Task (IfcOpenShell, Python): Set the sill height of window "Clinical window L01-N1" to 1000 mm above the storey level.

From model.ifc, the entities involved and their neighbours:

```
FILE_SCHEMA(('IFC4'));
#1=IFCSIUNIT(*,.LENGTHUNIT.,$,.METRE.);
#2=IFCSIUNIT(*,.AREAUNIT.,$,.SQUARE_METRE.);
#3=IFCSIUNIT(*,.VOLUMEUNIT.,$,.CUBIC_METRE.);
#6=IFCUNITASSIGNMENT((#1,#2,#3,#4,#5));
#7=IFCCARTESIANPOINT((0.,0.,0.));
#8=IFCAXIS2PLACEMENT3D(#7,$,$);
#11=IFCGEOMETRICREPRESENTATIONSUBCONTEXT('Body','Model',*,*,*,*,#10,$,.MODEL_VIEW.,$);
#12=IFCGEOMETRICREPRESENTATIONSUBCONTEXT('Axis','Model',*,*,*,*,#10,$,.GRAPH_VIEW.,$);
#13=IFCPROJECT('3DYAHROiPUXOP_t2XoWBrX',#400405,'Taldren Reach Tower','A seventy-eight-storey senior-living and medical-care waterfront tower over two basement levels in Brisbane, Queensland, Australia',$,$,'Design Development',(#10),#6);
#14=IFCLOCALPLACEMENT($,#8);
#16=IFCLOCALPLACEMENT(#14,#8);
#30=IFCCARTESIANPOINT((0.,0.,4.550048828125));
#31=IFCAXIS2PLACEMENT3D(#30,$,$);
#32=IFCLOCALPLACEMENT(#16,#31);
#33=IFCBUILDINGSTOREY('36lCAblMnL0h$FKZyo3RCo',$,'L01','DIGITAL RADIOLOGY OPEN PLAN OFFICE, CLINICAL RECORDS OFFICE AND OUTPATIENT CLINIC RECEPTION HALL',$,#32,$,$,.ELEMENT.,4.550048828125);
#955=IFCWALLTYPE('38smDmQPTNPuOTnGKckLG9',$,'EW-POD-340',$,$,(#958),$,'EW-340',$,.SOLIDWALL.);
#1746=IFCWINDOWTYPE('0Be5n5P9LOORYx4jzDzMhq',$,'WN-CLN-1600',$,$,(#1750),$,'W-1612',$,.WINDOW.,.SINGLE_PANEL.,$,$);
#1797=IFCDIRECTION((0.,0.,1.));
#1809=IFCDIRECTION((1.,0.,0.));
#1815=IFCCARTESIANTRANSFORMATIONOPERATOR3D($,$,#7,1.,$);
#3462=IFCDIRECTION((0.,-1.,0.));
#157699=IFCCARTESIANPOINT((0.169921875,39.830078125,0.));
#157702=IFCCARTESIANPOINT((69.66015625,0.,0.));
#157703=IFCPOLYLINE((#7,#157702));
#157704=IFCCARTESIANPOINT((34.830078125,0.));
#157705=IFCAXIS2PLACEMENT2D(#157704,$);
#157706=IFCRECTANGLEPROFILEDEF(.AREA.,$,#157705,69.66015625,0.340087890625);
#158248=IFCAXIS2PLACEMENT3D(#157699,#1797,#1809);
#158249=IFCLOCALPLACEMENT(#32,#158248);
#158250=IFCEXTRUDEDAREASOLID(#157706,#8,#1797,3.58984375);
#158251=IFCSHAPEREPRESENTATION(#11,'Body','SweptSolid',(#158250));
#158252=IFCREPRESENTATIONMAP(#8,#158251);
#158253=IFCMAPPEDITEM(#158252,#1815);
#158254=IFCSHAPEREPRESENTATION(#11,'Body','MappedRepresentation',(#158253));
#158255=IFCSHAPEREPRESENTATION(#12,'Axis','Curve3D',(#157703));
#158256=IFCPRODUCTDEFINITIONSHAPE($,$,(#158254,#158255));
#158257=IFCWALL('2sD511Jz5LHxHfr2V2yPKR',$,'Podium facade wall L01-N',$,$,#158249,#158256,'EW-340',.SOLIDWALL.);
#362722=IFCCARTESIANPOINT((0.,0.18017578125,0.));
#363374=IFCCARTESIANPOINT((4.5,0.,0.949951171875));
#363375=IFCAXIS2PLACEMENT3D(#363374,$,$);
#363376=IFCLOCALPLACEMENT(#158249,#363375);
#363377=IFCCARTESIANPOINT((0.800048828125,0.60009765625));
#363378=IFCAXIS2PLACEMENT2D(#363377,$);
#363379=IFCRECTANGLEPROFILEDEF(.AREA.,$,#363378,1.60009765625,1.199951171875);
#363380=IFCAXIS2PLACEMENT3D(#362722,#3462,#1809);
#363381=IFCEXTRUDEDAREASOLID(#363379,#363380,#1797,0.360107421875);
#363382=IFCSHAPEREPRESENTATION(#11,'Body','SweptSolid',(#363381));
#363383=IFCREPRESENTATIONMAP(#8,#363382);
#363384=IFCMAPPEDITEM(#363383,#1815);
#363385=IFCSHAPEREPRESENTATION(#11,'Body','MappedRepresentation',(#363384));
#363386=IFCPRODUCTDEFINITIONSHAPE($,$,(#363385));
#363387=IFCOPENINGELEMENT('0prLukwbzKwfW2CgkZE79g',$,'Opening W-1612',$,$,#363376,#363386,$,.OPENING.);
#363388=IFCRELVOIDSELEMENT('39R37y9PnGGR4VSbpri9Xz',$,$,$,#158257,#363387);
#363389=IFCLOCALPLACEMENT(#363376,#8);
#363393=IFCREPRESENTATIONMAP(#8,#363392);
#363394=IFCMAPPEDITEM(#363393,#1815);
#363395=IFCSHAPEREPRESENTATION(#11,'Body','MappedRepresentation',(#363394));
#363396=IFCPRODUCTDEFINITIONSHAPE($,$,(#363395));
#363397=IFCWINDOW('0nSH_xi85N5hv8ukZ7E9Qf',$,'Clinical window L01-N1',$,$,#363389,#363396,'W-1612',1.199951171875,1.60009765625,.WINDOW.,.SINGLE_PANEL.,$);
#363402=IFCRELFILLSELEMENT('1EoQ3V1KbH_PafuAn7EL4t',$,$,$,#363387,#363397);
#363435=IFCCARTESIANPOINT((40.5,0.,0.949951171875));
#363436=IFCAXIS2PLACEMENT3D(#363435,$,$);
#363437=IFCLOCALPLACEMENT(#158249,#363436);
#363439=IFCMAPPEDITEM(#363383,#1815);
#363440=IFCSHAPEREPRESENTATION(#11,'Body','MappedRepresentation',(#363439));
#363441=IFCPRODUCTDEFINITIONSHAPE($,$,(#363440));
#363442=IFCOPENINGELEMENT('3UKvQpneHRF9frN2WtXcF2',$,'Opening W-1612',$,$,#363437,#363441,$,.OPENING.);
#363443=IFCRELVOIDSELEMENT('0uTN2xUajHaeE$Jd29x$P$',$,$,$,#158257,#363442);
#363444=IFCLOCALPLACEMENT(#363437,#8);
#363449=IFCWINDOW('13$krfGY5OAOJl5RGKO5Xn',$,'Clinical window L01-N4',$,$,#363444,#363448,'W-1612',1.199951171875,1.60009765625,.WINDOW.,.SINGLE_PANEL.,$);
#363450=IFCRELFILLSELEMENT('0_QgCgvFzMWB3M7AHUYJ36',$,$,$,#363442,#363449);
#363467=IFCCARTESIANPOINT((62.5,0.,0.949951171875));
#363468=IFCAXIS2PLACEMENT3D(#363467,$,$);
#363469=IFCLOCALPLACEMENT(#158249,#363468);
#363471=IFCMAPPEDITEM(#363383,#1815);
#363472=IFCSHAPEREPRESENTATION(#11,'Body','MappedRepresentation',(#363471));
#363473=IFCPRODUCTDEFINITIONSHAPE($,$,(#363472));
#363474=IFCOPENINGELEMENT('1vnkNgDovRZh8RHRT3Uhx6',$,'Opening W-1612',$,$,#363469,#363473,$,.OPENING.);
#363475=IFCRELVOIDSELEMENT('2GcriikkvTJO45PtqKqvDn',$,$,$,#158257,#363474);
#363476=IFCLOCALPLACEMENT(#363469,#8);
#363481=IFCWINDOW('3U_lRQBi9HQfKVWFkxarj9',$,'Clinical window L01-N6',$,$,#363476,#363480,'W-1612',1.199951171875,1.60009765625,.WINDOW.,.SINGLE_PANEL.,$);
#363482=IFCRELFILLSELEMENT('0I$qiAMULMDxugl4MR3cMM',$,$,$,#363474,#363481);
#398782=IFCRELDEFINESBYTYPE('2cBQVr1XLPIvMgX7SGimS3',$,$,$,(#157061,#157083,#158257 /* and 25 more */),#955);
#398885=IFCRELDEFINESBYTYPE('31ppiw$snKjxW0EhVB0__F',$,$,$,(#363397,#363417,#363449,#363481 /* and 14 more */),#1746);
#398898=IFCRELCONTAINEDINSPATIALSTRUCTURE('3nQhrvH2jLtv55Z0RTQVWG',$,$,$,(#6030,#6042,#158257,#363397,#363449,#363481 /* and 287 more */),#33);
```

```python
import numpy as np
import ifcopenshell
import ifcopenshell.api.geometry
import ifcopenshell.geom
import ifcopenshell.util.element
import ifcopenshell.util.placement
import ifcopenshell.util.shape
import ifcopenshell.util.unit

model = ifcopenshell.open("model.ifc")
unit_scale = ifcopenshell.util.unit.calculate_unit_scale(model)

window = model.by_guid("0nSH_xi85N5hv8ukZ7E9Qf")
opening = window.FillsVoids[0].RelatingOpeningElement
storey = ifcopenshell.util.element.get_container(window, ifc_class="IfcBuildingStorey")
level = ifcopenshell.util.placement.get_local_placement(storey.ObjectPlacement)[2, 3]

# The opening's origin need not be at the sill, so measure its lowest point.
shape = ifcopenshell.geom.create_shape(ifcopenshell.geom.settings(), opening)
bottom = ifcopenshell.util.shape.get_shape_bottom_elevation(shape, shape.geometry) / unit_scale
dz = level + 1.0 - bottom

shift = np.array([0.0, 0.0, dz])
# The window is placed relative to its opening, so it follows when the opening moves.
matrix = ifcopenshell.util.placement.get_local_placement(opening.ObjectPlacement)
matrix[:3, 3] += shift
ifcopenshell.api.geometry.edit_object_placement(
    model, product=opening, matrix=matrix, is_si=False, should_transform_children=True
)

print(f"moved by {dz * unit_scale:+.3f} m")

model.write("model_updated.ifc")
```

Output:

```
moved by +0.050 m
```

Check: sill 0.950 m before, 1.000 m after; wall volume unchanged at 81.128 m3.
